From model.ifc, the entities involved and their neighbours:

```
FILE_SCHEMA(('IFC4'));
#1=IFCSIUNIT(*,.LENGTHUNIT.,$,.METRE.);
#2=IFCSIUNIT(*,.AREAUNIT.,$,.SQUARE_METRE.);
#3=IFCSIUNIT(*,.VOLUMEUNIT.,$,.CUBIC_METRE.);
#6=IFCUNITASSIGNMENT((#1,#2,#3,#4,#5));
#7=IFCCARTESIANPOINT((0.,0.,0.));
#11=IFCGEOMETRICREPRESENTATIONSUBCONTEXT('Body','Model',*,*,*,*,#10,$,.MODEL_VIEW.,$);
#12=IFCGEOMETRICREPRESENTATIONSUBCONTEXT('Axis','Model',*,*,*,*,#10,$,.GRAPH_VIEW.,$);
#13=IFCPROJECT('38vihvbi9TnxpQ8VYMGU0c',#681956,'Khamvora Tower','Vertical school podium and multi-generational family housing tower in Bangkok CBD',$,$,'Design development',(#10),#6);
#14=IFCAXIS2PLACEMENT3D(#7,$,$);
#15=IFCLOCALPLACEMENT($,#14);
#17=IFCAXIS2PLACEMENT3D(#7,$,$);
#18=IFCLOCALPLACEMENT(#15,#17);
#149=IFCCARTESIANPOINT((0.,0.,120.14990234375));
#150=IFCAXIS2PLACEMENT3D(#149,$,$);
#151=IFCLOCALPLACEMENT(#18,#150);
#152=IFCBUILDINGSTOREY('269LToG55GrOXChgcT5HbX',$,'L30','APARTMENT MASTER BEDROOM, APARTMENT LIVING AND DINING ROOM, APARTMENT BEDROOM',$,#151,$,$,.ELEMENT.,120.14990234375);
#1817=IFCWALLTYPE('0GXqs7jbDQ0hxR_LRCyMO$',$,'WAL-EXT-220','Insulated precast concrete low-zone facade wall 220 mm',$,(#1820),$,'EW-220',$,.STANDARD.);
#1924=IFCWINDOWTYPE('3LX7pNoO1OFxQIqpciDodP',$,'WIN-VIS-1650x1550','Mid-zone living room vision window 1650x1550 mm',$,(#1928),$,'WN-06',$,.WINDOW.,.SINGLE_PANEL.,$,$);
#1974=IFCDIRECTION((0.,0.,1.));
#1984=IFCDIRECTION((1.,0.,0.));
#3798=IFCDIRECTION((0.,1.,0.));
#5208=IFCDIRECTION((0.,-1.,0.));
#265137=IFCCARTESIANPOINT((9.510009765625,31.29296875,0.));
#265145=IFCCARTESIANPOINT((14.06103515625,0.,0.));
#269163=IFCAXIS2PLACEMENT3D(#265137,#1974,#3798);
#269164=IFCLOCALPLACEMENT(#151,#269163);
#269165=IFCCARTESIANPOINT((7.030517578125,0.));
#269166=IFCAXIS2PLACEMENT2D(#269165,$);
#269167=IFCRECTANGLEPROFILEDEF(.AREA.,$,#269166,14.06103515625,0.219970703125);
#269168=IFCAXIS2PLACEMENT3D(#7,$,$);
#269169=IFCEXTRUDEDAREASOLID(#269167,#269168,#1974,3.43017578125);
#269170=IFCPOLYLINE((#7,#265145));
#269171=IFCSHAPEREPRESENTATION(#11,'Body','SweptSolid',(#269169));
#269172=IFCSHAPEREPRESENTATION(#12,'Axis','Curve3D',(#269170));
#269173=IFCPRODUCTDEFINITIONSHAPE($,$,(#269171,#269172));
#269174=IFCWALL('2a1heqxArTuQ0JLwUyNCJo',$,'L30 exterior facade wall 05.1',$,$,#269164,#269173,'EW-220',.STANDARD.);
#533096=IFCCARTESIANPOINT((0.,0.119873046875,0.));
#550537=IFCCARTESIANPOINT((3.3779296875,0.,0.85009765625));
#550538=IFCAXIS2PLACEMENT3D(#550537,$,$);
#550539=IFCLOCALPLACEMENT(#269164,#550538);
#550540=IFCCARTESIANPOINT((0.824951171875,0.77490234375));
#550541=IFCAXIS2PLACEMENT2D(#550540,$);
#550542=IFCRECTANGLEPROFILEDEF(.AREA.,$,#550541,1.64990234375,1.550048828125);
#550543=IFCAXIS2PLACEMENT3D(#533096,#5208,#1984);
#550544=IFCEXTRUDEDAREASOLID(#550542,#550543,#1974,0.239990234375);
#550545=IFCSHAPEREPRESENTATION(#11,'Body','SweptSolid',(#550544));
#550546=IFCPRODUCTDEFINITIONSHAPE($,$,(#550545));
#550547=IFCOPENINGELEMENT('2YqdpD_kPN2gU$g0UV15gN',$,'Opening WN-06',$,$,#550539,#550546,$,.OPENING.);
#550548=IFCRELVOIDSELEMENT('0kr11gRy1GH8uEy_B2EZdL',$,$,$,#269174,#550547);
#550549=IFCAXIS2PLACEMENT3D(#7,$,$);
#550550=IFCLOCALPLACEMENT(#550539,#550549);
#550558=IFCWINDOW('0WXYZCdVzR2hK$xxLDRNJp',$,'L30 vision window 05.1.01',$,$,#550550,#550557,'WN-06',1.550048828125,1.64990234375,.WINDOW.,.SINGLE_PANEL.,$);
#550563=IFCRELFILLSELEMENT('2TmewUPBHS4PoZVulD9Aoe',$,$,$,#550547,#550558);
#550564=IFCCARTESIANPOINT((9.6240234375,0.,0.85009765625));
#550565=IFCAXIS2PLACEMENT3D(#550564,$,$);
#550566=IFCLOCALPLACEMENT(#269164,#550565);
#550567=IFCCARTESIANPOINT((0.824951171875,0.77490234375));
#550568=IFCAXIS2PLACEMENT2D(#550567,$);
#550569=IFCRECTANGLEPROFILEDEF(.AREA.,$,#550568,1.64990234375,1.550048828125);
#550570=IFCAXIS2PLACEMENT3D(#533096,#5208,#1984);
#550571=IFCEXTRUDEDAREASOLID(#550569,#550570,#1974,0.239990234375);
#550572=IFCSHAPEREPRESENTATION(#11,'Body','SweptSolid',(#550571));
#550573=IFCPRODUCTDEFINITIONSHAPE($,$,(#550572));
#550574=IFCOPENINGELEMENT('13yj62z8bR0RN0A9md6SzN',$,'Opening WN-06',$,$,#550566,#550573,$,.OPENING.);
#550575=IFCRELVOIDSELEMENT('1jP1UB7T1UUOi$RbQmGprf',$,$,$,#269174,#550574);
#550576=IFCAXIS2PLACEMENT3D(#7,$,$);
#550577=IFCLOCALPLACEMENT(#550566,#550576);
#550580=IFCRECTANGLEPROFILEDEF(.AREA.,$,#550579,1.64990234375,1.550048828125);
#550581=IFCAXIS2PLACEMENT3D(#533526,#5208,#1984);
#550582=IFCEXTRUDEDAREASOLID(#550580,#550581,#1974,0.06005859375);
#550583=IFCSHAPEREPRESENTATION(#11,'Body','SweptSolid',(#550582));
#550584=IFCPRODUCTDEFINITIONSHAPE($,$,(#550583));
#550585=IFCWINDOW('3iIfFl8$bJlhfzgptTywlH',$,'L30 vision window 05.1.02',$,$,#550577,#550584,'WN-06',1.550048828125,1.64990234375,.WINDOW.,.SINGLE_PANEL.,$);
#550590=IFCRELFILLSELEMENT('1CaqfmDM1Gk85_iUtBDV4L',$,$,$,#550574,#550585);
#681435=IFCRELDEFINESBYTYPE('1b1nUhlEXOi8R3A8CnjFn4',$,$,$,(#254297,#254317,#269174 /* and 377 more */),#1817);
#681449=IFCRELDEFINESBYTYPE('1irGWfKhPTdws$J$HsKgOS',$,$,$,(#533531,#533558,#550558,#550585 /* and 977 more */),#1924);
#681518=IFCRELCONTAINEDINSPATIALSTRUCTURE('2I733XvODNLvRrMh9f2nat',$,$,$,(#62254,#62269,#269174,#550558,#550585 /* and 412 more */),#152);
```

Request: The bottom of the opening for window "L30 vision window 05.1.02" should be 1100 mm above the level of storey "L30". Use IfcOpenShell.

```python
import numpy as np
import ifcopenshell
import ifcopenshell.api.geometry
import ifcopenshell.geom
import ifcopenshell.util.element
import ifcopenshell.util.placement
import ifcopenshell.util.shape
import ifcopenshell.util.unit

model = ifcopenshell.open("model.ifc")
unit_scale = ifcopenshell.util.unit.calculate_unit_scale(model)

window = model.by_guid("3iIfFl8$bJlhfzgptTywlH")
opening = window.FillsVoids[0].RelatingOpeningElement
storey = ifcopenshell.util.element.get_container(window, ifc_class="IfcBuildingStorey")
level = ifcopenshell.util.placement.get_local_placement(storey.ObjectPlacement)[2, 3]

# The opening's origin need not be at the sill, so measure its lowest point.
shape = ifcopenshell.geom.create_shape(ifcopenshell.geom.settings(), opening)
bottom = ifcopenshell.util.shape.get_shape_bottom_elevation(shape, shape.geometry) / unit_scale
dz = level + 1.1 - bottom

shift = np.array([0.0, 0.0, dz])
# The window is placed relative to its opening, so it follows when the opening moves.
matrix = ifcopenshell.util.placement.get_local_placement(opening.ObjectPlacement)
matrix[:3, 3] += shift
ifcopenshell.api.geometry.edit_object_placement(
    model, product=opening, matrix=matrix, is_si=False, should_transform_children=True
)

print(f"moved by {dz * unit_scale:+.3f} m")

model.write("model-out.ifc")
```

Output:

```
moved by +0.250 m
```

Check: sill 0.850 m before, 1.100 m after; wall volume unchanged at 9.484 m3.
